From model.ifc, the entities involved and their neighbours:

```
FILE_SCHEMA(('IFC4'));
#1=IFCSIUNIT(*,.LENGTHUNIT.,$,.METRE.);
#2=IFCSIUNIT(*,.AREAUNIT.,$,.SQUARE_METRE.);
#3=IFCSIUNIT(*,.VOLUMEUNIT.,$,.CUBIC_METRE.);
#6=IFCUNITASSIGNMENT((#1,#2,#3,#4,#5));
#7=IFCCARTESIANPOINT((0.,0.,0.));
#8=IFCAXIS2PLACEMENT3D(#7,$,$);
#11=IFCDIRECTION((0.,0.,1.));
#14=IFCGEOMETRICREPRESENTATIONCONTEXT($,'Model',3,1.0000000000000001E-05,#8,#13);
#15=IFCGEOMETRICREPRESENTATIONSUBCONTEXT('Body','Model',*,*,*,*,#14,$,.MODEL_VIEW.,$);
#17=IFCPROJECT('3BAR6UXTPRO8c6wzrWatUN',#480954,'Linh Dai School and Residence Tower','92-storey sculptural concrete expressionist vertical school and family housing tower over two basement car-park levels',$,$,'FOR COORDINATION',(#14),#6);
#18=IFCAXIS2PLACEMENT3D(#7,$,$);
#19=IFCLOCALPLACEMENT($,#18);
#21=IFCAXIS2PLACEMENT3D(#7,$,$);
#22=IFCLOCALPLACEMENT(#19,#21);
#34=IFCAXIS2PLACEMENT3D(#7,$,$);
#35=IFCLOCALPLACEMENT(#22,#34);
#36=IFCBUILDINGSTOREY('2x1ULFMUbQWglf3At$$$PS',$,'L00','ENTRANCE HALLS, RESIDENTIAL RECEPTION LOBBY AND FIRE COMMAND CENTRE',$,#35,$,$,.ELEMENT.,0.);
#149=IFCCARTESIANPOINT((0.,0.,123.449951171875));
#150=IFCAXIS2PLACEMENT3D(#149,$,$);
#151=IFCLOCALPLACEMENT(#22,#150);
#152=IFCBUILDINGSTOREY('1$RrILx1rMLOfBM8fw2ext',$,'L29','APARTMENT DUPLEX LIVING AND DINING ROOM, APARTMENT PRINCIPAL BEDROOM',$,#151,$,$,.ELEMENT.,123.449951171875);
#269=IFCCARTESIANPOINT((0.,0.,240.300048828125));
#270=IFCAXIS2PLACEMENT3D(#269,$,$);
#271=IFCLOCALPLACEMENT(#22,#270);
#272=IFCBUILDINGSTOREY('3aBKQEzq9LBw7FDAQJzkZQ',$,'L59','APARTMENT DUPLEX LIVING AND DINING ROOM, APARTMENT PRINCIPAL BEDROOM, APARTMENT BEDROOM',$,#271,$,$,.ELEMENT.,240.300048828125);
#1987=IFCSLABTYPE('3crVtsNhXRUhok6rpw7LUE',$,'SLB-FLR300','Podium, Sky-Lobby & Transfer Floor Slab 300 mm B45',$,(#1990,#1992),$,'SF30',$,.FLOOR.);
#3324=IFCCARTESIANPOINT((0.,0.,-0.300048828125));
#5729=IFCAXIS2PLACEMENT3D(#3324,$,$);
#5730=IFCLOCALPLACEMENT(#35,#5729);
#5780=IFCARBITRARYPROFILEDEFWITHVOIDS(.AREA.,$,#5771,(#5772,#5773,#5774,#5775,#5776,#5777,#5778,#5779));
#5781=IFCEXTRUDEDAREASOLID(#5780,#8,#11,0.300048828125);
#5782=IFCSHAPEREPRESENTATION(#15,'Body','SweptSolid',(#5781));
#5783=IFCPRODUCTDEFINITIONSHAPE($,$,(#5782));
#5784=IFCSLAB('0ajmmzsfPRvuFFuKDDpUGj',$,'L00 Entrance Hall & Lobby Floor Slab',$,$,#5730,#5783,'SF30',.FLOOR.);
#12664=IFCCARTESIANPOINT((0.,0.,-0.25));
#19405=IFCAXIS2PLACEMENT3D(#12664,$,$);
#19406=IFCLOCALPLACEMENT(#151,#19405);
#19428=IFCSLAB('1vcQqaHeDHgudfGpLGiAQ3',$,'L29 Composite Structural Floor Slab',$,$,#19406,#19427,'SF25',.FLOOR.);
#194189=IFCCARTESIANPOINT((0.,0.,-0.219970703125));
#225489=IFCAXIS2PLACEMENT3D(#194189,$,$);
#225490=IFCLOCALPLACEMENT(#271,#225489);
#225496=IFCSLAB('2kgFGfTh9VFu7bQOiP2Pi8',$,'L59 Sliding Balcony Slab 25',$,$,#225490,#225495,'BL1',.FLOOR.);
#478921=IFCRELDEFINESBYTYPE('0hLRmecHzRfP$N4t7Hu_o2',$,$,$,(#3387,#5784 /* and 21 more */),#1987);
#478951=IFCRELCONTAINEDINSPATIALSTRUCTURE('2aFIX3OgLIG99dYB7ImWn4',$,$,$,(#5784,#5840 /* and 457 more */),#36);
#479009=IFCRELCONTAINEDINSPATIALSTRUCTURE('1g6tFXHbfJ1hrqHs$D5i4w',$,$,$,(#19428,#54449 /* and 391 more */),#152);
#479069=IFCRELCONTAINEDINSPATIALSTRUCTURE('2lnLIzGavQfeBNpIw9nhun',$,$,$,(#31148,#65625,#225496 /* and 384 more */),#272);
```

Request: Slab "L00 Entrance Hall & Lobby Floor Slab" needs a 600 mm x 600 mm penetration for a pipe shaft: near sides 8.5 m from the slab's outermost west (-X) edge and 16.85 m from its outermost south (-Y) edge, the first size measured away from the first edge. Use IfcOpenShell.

```python
import numpy as np
import ifcopenshell
import ifcopenshell.api.feature
import ifcopenshell.api.geometry
import ifcopenshell.api.root
import ifcopenshell.geom
import ifcopenshell.util.placement
import ifcopenshell.util.representation
import ifcopenshell.util.shape
import ifcopenshell.util.unit

model = ifcopenshell.open("model.ifc")
unit_scale = ifcopenshell.util.unit.calculate_unit_scale(model)
settings = ifcopenshell.geom.settings()


def volume(element):
    """Net volume in cubic metres, openings subtracted."""
    shape = ifcopenshell.geom.create_shape(settings, element)
    return ifcopenshell.util.shape.get_volume(shape.geometry)


slab = model.by_guid("0ajmmzsfPRvuFFuKDDpUGj")
before = volume(slab)

# Extent in the slab's own axes, in metres. The edges named are its -X and -Y sides.
slab_shape = ifcopenshell.geom.create_shape(settings, slab)
vertices = ifcopenshell.util.shape.get_vertices(slab_shape.geometry)
x_min, y_min, bottom = vertices.min(axis=0)
top = vertices[:, 2].max()

opening = ifcopenshell.api.root.create_entity(model, ifc_class="IfcOpeningElement", name="Pipe shaft opening", predefined_type="OPENING")
context = ifcopenshell.util.representation.get_context(model, "Model", "Body", "MODEL_VIEW")
width, depth = 0.6, 0.6
outline = [(0.0, 0.0), (width, 0.0), (width, depth), (0.0, depth), (0.0, 0.0)]
# Overshoot both faces by 50 mm so the cut is clean.
shape = ifcopenshell.api.geometry.add_slab_representation(
    model, context=context, depth=top - bottom + 0.1, polyline=outline
)
ifcopenshell.api.geometry.assign_representation(model, product=opening, representation=shape)

matrix = ifcopenshell.util.placement.get_local_placement(slab.ObjectPlacement)
matrix[:, 3] = matrix @ np.append(np.array([x_min + 8.5, y_min + 16.85, bottom - 0.05]) / unit_scale, 1.0)
ifcopenshell.api.geometry.edit_object_placement(model, product=opening, matrix=matrix, is_si=False)
ifcopenshell.api.feature.add_feature(model, feature=opening, element=slab)

after = volume(slab)

print(f"slab volume {before:.3f} -> {after:.3f} m3")

model.write("model_rev.ifc")
```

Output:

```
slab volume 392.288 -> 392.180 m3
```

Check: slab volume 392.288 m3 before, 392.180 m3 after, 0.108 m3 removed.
